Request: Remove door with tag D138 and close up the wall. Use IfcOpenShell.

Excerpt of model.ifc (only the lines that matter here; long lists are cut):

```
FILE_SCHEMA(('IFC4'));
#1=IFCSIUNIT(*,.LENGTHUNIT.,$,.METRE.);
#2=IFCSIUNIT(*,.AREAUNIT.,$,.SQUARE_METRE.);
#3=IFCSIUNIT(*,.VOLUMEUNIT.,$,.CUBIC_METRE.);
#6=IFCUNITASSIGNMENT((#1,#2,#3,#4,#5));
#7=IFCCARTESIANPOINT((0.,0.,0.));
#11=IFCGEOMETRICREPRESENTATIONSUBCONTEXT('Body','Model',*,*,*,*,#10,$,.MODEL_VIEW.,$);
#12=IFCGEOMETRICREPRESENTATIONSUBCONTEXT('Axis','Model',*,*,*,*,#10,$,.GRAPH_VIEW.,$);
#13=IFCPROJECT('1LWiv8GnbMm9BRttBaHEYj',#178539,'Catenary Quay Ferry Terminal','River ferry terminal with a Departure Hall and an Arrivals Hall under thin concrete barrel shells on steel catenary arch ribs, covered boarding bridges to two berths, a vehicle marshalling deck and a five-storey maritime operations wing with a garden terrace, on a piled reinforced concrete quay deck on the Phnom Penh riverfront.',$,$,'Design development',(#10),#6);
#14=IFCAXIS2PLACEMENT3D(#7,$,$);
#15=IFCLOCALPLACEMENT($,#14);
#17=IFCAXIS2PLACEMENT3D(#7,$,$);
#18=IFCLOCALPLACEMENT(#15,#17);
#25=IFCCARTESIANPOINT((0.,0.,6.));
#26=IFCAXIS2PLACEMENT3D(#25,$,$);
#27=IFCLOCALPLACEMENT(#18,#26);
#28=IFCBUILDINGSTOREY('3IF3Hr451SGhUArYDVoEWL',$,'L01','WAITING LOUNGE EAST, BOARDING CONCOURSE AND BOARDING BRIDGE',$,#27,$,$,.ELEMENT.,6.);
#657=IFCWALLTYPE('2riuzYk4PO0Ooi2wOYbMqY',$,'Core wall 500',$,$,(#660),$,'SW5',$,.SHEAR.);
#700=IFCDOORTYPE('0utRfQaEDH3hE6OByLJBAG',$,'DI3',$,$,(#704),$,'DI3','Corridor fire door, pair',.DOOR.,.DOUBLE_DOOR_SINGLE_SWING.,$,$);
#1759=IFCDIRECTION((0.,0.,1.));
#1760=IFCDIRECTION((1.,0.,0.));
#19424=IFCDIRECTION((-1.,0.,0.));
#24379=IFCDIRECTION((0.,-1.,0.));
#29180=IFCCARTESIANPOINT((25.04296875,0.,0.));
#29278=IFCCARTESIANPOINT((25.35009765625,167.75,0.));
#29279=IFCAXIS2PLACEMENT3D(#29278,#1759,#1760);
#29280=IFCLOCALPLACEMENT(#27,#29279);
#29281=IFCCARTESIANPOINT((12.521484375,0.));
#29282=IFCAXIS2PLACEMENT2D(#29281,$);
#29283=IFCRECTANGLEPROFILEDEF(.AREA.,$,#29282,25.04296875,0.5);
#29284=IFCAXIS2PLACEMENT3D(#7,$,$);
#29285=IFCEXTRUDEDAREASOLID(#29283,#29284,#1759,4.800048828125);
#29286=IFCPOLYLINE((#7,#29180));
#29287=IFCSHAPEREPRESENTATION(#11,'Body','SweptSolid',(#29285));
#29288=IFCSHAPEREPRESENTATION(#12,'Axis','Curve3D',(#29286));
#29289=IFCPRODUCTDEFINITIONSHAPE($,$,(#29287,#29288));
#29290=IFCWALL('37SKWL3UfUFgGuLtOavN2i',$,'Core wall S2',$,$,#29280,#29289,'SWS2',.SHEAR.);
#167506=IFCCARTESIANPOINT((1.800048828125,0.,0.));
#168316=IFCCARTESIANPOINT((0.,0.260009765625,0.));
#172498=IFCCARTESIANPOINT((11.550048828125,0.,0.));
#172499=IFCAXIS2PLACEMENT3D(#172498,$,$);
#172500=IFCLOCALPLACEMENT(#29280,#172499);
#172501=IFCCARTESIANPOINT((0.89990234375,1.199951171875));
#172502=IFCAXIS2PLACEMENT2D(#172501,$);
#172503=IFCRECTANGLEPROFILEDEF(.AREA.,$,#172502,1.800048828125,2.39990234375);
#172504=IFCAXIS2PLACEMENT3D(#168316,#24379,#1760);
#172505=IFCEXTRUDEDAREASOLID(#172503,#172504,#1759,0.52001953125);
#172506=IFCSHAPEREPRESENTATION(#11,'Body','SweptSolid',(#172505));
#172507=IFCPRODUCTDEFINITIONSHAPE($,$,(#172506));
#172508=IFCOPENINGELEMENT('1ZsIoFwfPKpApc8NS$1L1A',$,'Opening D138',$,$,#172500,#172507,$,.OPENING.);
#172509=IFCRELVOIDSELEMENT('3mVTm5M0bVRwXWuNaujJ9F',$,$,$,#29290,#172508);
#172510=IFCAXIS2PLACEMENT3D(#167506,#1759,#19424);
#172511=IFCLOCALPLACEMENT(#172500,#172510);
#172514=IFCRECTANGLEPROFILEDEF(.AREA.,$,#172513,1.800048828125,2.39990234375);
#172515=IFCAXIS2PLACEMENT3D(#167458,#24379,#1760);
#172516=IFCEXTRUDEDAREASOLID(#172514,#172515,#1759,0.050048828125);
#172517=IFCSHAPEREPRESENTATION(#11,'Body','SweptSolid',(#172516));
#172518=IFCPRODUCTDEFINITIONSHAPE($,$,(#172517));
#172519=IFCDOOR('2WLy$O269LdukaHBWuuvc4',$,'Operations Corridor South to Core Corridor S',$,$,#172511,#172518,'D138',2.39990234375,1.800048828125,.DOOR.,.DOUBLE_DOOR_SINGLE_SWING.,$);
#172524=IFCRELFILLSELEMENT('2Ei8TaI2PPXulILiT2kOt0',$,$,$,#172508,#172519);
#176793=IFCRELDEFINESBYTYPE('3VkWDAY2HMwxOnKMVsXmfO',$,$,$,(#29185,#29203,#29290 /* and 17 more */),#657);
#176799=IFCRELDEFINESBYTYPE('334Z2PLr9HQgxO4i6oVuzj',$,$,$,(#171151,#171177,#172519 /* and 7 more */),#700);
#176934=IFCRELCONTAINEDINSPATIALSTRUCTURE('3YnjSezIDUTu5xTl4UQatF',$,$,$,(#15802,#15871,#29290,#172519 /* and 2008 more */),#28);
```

```python
import ifcopenshell
import ifcopenshell.api.feature
import ifcopenshell.api.root
import ifcopenshell.geom
import ifcopenshell.util.shape

model = ifcopenshell.open("model.ifc")
settings = ifcopenshell.geom.settings()


def volume(element):
    """Net volume in cubic metres, openings subtracted."""
    shape = ifcopenshell.geom.create_shape(settings, element)
    return ifcopenshell.util.shape.get_volume(shape.geometry)


door = model.by_guid("2WLy$O269LdukaHBWuuvc4")
opening = door.FillsVoids[0].RelatingOpeningElement
wall = opening.VoidsElements[0].RelatingBuildingElement
before = volume(wall)

ifcopenshell.api.root.remove_product(model, product=door)
ifcopenshell.api.feature.remove_feature(model, feature=opening)

after = volume(wall)

print(f"wall volume {before:.3f} -> {after:.3f} m3")

model.write("model_rev.ifc")
```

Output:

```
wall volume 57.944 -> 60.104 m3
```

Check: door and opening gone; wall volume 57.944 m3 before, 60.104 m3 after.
